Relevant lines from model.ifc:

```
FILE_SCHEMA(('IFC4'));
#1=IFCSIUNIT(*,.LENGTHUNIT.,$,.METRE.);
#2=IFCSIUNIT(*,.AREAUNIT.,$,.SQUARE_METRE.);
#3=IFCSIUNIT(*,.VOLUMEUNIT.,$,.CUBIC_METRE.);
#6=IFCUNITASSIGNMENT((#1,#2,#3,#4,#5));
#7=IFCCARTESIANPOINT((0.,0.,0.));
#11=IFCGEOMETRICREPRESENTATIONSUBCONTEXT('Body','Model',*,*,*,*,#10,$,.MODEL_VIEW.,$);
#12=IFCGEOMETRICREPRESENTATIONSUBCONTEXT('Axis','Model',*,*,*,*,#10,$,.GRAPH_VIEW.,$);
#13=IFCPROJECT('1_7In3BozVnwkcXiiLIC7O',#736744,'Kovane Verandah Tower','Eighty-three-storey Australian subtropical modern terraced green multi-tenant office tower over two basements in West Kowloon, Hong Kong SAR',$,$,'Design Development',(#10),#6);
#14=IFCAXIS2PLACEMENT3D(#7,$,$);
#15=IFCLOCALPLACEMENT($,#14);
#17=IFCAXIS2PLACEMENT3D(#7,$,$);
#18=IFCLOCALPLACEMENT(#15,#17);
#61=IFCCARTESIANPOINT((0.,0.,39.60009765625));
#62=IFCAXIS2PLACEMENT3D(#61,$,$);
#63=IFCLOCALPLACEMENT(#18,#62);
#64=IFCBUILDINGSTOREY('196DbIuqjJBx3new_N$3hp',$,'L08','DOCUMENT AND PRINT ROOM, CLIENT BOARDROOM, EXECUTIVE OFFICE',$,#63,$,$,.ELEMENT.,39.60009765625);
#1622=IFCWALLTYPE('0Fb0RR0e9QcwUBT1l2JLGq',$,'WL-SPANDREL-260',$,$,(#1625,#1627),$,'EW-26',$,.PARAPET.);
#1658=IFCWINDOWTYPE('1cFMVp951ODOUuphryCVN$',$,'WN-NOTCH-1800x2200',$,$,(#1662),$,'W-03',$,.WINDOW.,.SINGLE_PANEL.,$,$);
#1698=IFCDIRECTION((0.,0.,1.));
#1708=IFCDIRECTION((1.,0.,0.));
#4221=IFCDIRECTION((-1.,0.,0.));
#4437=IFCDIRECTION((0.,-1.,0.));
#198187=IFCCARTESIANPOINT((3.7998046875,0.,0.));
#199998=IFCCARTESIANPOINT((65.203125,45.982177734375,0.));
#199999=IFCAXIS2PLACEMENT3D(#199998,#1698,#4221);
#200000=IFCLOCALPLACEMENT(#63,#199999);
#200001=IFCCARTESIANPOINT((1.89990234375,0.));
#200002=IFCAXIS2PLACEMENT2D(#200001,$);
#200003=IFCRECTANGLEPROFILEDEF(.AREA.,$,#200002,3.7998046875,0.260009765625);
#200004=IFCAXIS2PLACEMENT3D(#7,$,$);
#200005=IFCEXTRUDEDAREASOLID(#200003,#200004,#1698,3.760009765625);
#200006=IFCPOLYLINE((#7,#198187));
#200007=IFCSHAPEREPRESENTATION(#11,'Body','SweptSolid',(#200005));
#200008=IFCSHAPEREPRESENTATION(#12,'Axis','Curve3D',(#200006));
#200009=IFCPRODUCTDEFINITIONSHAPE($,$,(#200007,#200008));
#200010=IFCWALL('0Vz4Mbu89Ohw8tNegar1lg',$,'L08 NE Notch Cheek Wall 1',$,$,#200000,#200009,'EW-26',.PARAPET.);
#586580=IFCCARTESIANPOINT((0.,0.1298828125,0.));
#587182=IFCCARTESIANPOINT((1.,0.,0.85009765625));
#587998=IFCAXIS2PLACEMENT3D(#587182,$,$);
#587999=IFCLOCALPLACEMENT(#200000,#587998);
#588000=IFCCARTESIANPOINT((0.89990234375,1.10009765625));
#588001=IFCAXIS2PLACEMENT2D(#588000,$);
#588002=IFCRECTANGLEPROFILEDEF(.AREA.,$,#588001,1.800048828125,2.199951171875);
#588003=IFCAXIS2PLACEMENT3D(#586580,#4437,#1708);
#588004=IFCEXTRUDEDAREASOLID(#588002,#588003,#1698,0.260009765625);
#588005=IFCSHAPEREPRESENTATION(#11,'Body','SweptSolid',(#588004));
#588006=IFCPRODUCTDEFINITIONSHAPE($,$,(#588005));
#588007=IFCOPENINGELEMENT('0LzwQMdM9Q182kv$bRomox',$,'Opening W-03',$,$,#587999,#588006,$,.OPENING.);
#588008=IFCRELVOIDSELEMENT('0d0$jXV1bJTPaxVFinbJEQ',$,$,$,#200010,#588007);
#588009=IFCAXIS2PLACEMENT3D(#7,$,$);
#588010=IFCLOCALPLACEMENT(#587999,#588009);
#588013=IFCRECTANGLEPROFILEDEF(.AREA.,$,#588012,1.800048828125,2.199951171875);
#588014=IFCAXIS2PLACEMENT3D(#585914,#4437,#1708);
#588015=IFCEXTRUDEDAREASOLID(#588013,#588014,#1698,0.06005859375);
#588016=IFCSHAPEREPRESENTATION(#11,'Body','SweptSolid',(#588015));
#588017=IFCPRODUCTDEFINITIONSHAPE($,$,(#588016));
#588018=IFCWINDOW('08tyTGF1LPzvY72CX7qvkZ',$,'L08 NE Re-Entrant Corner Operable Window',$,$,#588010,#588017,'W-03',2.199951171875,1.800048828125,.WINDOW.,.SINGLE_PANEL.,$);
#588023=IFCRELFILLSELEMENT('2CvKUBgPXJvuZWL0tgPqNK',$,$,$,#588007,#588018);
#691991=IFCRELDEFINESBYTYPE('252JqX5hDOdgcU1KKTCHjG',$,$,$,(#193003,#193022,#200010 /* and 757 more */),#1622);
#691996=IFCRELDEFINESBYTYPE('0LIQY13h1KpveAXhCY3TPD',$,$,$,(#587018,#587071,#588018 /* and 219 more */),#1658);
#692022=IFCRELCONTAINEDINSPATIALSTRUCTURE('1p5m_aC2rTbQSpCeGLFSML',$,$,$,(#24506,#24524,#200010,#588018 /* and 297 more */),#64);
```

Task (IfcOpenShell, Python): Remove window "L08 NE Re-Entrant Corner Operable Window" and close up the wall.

```python
import ifcopenshell
import ifcopenshell.api.feature
import ifcopenshell.api.root
import ifcopenshell.geom
import ifcopenshell.util.shape

model = ifcopenshell.open("model.ifc")
settings = ifcopenshell.geom.settings()


def volume(element):
    """Net volume in cubic metres, openings subtracted."""
    shape = ifcopenshell.geom.create_shape(settings, element)
    return ifcopenshell.util.shape.get_volume(shape.geometry)


window = model.by_id(588018)
opening = window.FillsVoids[0].RelatingOpeningElement
wall = opening.VoidsElements[0].RelatingBuildingElement
before = volume(wall)

ifcopenshell.api.root.remove_product(model, product=window)
ifcopenshell.api.feature.remove_feature(model, feature=opening)

after = volume(wall)

print(f"wall volume {before:.3f} -> {after:.3f} m3")

model.write("model_v2.ifc")
```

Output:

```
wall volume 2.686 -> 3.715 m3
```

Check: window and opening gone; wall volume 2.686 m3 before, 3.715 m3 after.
